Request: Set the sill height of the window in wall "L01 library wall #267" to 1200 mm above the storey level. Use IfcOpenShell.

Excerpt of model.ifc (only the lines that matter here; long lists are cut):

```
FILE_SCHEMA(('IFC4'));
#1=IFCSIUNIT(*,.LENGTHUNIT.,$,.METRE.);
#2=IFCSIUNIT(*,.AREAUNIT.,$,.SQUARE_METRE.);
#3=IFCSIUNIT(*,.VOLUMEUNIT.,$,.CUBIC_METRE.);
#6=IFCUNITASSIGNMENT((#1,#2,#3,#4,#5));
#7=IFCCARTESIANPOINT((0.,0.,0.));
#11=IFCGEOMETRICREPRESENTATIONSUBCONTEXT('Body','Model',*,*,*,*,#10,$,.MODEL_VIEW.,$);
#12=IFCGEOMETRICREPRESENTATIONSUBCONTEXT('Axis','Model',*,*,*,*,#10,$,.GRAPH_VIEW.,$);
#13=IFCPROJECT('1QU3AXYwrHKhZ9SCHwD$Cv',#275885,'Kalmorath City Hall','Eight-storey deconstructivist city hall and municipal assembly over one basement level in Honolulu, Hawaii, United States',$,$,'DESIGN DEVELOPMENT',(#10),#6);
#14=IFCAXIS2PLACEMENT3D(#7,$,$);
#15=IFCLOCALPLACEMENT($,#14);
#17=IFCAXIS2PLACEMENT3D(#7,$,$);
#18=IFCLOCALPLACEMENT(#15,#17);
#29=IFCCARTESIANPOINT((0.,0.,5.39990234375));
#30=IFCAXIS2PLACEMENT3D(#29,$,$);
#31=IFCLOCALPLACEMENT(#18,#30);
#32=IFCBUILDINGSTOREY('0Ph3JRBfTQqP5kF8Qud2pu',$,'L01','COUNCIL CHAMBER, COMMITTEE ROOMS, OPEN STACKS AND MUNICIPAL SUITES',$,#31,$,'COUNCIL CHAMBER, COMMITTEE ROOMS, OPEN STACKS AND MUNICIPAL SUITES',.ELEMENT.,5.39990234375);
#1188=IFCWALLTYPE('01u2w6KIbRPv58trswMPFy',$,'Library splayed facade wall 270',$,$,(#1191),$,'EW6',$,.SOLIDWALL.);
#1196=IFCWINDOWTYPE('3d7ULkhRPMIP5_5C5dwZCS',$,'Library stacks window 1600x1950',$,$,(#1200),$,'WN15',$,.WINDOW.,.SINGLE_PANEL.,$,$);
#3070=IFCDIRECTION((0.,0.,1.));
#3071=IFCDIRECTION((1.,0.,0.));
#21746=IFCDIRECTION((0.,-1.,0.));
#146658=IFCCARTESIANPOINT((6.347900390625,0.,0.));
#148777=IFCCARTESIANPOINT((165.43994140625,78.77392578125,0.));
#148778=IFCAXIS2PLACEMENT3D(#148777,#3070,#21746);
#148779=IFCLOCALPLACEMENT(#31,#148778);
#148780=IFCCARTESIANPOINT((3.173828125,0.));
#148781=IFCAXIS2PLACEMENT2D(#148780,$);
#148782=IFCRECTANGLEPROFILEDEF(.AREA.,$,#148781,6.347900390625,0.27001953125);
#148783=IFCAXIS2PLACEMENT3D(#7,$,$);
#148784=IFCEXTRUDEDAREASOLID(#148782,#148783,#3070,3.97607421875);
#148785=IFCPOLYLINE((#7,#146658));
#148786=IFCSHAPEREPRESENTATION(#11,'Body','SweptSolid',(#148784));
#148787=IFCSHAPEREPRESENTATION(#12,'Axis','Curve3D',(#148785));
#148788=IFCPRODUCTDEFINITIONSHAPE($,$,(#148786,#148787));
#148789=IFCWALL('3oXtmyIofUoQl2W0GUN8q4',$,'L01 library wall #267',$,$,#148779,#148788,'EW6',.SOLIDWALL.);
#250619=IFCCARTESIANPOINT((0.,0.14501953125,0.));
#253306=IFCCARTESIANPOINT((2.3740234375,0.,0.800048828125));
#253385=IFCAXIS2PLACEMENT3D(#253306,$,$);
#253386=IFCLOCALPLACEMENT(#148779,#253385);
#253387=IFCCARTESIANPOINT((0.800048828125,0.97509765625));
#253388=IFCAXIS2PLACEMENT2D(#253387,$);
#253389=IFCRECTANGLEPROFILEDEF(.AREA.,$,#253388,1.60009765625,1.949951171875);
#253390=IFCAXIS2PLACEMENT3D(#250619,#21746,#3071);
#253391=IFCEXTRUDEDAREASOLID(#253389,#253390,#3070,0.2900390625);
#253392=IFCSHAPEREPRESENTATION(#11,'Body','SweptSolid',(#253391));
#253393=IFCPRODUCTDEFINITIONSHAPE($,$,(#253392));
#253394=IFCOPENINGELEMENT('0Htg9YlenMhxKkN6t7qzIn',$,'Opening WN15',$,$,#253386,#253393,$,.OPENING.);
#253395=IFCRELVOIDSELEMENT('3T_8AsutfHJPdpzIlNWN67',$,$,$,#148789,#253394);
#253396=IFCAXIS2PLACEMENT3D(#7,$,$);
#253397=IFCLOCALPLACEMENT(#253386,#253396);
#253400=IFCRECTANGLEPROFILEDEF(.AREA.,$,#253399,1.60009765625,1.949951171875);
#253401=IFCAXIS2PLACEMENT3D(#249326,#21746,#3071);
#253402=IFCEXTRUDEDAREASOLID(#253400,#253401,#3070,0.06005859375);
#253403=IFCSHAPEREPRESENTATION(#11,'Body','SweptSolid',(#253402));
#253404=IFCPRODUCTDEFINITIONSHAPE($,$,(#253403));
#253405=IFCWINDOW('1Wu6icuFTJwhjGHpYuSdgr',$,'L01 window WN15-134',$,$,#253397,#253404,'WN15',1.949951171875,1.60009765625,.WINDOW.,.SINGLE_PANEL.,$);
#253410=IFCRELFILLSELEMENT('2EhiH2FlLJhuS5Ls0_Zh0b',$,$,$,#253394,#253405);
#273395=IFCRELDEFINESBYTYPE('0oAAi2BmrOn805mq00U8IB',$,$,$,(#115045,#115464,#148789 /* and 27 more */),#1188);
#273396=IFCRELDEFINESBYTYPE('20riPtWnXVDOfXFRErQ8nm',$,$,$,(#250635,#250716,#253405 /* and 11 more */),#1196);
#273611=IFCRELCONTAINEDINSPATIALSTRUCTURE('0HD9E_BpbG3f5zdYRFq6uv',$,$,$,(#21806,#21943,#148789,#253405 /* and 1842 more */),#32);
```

```python
import numpy as np
import ifcopenshell
import ifcopenshell.api.geometry
import ifcopenshell.geom
import ifcopenshell.util.element
import ifcopenshell.util.placement
import ifcopenshell.util.shape
import ifcopenshell.util.unit

model = ifcopenshell.open("model.ifc")
unit_scale = ifcopenshell.util.unit.calculate_unit_scale(model)

window = model.by_guid("1Wu6icuFTJwhjGHpYuSdgr")
opening = window.FillsVoids[0].RelatingOpeningElement
storey = ifcopenshell.util.element.get_container(window, ifc_class="IfcBuildingStorey")
level = ifcopenshell.util.placement.get_local_placement(storey.ObjectPlacement)[2, 3]

# The opening's origin need not be at the sill, so measure its lowest point.
shape = ifcopenshell.geom.create_shape(ifcopenshell.geom.settings(), opening)
bottom = ifcopenshell.util.shape.get_shape_bottom_elevation(shape, shape.geometry) / unit_scale
dz = level + 1.2 - bottom

shift = np.array([0.0, 0.0, dz])
# The window is placed relative to its opening, so it follows when the opening moves.
matrix = ifcopenshell.util.placement.get_local_placement(opening.ObjectPlacement)
matrix[:3, 3] += shift
ifcopenshell.api.geometry.edit_object_placement(
    model, product=opening, matrix=matrix, is_si=False, should_transform_children=True
)

print(f"moved by {dz * unit_scale:+.3f} m")

model.write("model_v2.ifc")
```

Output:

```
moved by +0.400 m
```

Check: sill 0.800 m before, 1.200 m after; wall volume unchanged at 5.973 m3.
